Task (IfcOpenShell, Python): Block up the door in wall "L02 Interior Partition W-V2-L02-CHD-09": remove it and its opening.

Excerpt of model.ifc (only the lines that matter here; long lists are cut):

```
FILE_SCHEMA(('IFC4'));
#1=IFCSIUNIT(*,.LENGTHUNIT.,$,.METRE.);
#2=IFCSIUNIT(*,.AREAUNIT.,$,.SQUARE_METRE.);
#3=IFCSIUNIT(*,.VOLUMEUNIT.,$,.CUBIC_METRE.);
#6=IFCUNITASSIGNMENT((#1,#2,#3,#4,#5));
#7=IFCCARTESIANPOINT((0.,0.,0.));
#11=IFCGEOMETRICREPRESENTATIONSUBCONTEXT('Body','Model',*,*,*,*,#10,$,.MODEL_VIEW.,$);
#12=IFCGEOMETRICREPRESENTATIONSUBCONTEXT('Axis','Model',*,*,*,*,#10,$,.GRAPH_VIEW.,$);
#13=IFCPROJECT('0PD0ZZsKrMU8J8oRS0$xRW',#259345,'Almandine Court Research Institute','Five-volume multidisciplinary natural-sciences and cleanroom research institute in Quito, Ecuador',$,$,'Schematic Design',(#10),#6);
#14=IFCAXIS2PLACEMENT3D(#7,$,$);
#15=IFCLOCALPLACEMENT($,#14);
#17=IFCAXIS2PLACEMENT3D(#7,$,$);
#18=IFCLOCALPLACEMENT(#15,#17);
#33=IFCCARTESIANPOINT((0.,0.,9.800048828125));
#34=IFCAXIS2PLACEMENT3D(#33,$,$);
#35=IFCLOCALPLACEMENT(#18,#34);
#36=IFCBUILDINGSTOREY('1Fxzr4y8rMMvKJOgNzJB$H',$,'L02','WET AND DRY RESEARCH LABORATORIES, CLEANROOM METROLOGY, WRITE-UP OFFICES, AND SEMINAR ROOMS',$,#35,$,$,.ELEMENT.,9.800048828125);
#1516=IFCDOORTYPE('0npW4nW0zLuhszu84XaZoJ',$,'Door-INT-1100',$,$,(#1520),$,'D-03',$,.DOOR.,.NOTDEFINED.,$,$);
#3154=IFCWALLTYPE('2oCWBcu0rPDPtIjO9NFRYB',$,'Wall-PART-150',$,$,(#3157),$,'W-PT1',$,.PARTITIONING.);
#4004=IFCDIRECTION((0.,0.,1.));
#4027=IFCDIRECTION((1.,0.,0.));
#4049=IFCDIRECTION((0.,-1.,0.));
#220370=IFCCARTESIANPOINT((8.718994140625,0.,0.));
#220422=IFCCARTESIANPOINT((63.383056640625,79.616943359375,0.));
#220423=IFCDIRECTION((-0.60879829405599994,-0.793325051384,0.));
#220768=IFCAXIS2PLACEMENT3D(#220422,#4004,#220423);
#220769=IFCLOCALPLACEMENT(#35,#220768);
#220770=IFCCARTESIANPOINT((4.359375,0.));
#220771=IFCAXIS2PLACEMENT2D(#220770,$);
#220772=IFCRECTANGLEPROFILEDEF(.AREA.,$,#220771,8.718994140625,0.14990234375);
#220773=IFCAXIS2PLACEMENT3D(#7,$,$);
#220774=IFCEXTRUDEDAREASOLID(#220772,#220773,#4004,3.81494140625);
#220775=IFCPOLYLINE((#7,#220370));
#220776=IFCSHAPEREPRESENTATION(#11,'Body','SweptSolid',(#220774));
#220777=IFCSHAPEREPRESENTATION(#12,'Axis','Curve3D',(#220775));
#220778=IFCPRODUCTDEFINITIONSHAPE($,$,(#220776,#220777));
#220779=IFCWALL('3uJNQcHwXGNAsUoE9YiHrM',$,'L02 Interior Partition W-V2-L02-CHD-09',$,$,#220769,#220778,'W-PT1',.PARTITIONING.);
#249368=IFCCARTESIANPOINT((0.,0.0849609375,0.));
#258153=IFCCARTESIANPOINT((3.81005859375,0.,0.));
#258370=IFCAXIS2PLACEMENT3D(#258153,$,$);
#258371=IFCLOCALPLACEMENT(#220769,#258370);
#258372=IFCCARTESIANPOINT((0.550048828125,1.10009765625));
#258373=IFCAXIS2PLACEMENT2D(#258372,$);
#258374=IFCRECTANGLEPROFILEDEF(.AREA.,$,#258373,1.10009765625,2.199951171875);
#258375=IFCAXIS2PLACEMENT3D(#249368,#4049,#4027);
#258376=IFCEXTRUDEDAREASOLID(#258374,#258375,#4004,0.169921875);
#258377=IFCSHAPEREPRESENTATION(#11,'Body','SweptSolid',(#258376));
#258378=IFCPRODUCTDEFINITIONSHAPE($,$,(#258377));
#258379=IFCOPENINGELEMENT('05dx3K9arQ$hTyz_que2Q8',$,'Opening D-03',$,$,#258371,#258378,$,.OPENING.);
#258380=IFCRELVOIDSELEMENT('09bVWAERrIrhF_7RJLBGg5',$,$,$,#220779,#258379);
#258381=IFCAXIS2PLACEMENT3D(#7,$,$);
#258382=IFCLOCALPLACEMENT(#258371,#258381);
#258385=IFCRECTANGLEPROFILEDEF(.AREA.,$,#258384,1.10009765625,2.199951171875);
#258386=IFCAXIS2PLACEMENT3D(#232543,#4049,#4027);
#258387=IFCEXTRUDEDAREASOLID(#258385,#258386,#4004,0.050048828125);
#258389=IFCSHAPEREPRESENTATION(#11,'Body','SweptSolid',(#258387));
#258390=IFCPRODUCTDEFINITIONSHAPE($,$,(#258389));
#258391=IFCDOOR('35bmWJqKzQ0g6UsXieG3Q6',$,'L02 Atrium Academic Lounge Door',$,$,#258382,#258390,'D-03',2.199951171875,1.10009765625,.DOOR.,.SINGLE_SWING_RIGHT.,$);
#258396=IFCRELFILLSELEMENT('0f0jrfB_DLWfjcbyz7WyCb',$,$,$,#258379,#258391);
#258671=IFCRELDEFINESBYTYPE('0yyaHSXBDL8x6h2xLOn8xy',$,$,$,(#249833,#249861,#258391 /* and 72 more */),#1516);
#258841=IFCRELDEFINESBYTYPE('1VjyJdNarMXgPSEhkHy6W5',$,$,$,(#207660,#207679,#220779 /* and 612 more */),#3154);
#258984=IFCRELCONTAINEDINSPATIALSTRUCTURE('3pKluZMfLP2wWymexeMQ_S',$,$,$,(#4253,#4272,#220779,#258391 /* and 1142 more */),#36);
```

```python
import ifcopenshell
import ifcopenshell.api.feature
import ifcopenshell.api.root
import ifcopenshell.geom
import ifcopenshell.util.shape

model = ifcopenshell.open("model.ifc")
settings = ifcopenshell.geom.settings()


def volume(element):
    """Net volume in cubic metres, openings subtracted."""
    shape = ifcopenshell.geom.create_shape(settings, element)
    return ifcopenshell.util.shape.get_volume(shape.geometry)


door = model.by_guid("35bmWJqKzQ0g6UsXieG3Q6")
opening = door.FillsVoids[0].RelatingOpeningElement
wall = opening.VoidsElements[0].RelatingBuildingElement
before = volume(wall)

ifcopenshell.api.root.remove_product(model, product=door)
ifcopenshell.api.feature.remove_feature(model, feature=opening)

after = volume(wall)

print(f"wall volume {before:.3f} -> {after:.3f} m3")

model.write("model_v2.ifc")
```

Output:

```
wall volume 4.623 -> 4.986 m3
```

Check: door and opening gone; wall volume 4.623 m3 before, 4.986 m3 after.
